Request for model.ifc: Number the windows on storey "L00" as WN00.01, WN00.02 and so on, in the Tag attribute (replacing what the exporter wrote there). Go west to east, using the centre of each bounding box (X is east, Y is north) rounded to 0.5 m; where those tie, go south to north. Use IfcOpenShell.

First a look at what the model holds.

```python
import ifcopenshell
import ifcopenshell.util.element
import ifcopenshell.util.placement

model = ifcopenshell.open("model.ifc")
print(model.schema)
storey = next(s for s in model.by_type("IfcBuildingStorey") if s.Name == "L00")
windows = [e for e in ifcopenshell.util.element.get_decomposition(storey) if e.is_a("IfcWindow")]
for e in sorted(windows, key=lambda e: e.id()):
    origin = ifcopenshell.util.placement.get_local_placement(e.ObjectPlacement)[:3, 3]
    print(e.id(), e.Tag, e.Name, origin.round(2) + 0.0, sep=" | ")
```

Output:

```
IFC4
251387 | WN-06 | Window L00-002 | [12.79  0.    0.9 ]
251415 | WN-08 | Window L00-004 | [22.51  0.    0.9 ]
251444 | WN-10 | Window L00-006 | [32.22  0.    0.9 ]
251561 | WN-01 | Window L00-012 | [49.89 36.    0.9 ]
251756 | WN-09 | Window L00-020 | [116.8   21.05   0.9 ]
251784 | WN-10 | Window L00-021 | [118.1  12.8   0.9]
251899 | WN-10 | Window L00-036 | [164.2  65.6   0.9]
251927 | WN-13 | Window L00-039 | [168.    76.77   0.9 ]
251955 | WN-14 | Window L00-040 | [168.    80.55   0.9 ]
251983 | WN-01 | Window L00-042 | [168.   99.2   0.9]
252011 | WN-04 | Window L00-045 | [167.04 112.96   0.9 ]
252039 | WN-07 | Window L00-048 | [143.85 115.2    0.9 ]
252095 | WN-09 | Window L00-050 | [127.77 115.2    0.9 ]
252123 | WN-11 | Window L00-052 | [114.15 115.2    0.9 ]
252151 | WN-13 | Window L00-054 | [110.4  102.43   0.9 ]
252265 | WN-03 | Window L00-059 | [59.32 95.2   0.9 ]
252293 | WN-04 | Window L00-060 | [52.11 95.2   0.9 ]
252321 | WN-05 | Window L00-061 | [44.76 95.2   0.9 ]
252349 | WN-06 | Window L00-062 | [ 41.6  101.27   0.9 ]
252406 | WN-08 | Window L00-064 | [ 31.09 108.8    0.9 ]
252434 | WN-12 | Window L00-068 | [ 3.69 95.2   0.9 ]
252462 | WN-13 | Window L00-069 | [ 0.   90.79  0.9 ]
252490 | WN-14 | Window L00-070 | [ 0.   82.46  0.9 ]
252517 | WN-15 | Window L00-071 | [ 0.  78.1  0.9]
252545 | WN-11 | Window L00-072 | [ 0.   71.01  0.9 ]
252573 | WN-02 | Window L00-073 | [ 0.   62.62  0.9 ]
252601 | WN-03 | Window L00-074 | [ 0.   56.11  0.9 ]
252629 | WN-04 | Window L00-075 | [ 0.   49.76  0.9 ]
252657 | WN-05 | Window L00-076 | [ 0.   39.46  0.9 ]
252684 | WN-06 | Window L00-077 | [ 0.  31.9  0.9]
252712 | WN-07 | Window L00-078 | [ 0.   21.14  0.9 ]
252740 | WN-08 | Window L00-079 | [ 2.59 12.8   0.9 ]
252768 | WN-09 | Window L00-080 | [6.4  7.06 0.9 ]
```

```python
import ifcopenshell
import ifcopenshell.geom
import ifcopenshell.util.element
import ifcopenshell.util.shape

model = ifcopenshell.open("model.ifc")
settings = ifcopenshell.geom.settings()
settings.set("use-world-coords", True)


def centre(element):
    shape = ifcopenshell.geom.create_shape(settings, element)
    return ifcopenshell.util.shape.get_bbox_centroid(shape.geometry)


storey = next(s for s in model.by_type("IfcBuildingStorey") if s.Name == "L00")
windows = [e for e in ifcopenshell.util.element.get_decomposition(storey) if e.is_a("IfcWindow")]

# Insertion points can sit at a corner or the storey origin, so sort by the geometry (in metres).
centres = {e: centre(e) for e in windows}
windows.sort(key=lambda e: (round(centres[e][0] / 0.5), centres[e][1]))

for i, e in enumerate(windows, start=1):
    number = f"WN00.{i:02d}"
    e.Tag = number
    print(e.id(), number)

model.write("model_v2.ifc")
```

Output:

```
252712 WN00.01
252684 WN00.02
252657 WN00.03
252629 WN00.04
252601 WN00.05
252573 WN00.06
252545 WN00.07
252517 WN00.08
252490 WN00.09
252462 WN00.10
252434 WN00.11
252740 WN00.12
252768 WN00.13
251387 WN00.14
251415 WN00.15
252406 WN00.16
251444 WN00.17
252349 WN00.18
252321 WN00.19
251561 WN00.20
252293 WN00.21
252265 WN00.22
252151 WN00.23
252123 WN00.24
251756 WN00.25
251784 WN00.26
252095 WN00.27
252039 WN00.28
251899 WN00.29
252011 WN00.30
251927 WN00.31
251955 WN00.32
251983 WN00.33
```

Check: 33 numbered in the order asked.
